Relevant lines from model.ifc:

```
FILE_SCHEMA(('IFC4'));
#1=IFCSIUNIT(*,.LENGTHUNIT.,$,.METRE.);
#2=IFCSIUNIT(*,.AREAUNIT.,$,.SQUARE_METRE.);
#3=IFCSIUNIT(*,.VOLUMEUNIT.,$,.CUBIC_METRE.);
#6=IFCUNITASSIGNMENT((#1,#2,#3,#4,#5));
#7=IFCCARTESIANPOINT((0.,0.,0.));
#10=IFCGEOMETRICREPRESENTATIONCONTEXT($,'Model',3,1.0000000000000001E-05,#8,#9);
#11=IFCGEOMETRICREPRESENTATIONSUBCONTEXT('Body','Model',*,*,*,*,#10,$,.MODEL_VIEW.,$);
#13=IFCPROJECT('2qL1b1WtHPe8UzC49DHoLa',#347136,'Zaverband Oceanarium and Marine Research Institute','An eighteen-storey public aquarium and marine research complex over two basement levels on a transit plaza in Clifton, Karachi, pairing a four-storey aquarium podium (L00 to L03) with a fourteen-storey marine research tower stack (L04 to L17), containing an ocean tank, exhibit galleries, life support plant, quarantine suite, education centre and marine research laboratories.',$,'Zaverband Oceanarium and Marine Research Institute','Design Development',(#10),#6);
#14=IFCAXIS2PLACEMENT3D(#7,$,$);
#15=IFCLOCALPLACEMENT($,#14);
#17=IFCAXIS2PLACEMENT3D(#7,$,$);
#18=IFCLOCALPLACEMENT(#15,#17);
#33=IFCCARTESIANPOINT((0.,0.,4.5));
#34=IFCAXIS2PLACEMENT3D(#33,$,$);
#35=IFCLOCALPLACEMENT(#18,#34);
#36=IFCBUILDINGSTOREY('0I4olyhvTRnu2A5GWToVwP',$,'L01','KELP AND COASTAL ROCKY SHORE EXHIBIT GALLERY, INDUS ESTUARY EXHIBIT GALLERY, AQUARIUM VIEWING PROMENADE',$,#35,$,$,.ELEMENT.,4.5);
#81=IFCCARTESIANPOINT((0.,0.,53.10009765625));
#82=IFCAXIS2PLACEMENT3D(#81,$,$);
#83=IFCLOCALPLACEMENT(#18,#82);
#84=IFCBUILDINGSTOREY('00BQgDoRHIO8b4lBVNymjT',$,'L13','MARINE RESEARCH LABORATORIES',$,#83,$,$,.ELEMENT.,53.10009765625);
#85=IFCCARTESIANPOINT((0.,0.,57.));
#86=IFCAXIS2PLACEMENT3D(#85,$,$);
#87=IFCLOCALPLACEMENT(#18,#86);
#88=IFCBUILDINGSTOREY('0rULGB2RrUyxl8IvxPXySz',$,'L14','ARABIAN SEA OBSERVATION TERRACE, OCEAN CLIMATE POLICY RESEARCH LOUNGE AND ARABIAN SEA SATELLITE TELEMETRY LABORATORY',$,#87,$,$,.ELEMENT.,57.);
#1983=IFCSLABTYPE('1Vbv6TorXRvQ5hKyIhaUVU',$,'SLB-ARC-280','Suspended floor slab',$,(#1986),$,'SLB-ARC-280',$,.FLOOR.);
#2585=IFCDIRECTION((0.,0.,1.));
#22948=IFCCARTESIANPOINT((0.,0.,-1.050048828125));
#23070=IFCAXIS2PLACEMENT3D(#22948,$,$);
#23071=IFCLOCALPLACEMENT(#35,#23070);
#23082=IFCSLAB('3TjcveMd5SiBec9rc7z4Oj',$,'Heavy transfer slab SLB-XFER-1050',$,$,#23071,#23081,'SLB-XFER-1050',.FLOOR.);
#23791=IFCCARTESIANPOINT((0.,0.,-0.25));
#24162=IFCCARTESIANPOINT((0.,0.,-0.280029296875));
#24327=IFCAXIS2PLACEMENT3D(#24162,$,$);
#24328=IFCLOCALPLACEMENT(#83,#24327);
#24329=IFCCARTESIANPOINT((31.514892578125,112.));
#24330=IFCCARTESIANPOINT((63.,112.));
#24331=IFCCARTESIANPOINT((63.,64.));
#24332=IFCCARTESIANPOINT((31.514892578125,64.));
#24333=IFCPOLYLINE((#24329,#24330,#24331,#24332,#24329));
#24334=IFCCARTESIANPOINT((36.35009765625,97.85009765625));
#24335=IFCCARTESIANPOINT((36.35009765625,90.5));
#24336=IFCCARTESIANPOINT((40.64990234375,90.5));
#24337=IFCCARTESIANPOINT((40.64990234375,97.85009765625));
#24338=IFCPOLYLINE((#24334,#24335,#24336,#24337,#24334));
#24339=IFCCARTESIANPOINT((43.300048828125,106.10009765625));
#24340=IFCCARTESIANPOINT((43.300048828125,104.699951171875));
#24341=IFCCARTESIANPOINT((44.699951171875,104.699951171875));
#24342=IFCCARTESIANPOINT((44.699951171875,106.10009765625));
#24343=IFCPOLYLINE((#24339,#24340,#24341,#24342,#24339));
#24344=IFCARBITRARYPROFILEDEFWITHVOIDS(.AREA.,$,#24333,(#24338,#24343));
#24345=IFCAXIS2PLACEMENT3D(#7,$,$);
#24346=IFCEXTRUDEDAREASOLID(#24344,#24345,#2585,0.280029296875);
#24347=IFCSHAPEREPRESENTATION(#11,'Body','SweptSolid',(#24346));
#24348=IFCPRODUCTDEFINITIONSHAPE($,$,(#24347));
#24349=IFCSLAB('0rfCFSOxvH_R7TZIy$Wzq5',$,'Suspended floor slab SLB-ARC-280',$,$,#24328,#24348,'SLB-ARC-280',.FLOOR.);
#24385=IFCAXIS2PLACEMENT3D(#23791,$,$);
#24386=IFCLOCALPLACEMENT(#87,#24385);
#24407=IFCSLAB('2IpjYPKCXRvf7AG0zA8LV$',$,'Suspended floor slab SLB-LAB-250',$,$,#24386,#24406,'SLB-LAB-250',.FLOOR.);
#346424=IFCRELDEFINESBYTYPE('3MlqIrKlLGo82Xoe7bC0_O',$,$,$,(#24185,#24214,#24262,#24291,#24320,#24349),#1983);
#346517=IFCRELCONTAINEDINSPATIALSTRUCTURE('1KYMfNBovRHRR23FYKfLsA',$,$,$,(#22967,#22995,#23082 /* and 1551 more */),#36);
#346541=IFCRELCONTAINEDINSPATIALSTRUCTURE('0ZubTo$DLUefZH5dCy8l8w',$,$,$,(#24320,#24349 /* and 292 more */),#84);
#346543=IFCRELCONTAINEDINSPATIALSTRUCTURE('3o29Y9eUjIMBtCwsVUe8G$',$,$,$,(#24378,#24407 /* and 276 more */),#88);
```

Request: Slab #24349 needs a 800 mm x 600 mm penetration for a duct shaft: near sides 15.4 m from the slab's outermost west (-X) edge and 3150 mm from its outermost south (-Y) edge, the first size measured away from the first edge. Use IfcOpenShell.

```python
import numpy as np
import ifcopenshell
import ifcopenshell.api.feature
import ifcopenshell.api.geometry
import ifcopenshell.api.root
import ifcopenshell.geom
import ifcopenshell.util.placement
import ifcopenshell.util.representation
import ifcopenshell.util.shape
import ifcopenshell.util.unit

model = ifcopenshell.open("model.ifc")
unit_scale = ifcopenshell.util.unit.calculate_unit_scale(model)
settings = ifcopenshell.geom.settings()


def volume(element):
    """Net volume in cubic metres, openings subtracted."""
    shape = ifcopenshell.geom.create_shape(settings, element)
    return ifcopenshell.util.shape.get_volume(shape.geometry)


slab = model.by_guid("0rfCFSOxvH_R7TZIy$Wzq5")
before = volume(slab)

# Extent in the slab's own axes, in metres. The edges named are its -X and -Y sides.
slab_shape = ifcopenshell.geom.create_shape(settings, slab)
vertices = ifcopenshell.util.shape.get_vertices(slab_shape.geometry)
x_min, y_min, bottom = vertices.min(axis=0)
top = vertices[:, 2].max()

opening = ifcopenshell.api.root.create_entity(model, ifc_class="IfcOpeningElement", name="Duct shaft opening", predefined_type="OPENING")
context = ifcopenshell.util.representation.get_context(model, "Model", "Body", "MODEL_VIEW")
width, depth = 0.8, 0.6
outline = [(0.0, 0.0), (width, 0.0), (width, depth), (0.0, depth), (0.0, 0.0)]
# Overshoot both faces by 50 mm so the cut is clean.
shape = ifcopenshell.api.geometry.add_slab_representation(
    model, context=context, depth=top - bottom + 0.1, polyline=outline
)
ifcopenshell.api.geometry.assign_representation(model, product=opening, representation=shape)

matrix = ifcopenshell.util.placement.get_local_placement(slab.ObjectPlacement)
matrix[:, 3] = matrix @ np.append(np.array([x_min + 15.4, y_min + 3.15, bottom - 0.05]) / unit_scale, 1.0)
ifcopenshell.api.geometry.edit_object_placement(model, product=opening, matrix=matrix, is_si=False)
ifcopenshell.api.feature.add_feature(model, feature=opening, element=slab)

after = volume(slab)

print(f"slab volume {before:.3f} -> {after:.3f} m3")

model.write("model_updated.ifc")
```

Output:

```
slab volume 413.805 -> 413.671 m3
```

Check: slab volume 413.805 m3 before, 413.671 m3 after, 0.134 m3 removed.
